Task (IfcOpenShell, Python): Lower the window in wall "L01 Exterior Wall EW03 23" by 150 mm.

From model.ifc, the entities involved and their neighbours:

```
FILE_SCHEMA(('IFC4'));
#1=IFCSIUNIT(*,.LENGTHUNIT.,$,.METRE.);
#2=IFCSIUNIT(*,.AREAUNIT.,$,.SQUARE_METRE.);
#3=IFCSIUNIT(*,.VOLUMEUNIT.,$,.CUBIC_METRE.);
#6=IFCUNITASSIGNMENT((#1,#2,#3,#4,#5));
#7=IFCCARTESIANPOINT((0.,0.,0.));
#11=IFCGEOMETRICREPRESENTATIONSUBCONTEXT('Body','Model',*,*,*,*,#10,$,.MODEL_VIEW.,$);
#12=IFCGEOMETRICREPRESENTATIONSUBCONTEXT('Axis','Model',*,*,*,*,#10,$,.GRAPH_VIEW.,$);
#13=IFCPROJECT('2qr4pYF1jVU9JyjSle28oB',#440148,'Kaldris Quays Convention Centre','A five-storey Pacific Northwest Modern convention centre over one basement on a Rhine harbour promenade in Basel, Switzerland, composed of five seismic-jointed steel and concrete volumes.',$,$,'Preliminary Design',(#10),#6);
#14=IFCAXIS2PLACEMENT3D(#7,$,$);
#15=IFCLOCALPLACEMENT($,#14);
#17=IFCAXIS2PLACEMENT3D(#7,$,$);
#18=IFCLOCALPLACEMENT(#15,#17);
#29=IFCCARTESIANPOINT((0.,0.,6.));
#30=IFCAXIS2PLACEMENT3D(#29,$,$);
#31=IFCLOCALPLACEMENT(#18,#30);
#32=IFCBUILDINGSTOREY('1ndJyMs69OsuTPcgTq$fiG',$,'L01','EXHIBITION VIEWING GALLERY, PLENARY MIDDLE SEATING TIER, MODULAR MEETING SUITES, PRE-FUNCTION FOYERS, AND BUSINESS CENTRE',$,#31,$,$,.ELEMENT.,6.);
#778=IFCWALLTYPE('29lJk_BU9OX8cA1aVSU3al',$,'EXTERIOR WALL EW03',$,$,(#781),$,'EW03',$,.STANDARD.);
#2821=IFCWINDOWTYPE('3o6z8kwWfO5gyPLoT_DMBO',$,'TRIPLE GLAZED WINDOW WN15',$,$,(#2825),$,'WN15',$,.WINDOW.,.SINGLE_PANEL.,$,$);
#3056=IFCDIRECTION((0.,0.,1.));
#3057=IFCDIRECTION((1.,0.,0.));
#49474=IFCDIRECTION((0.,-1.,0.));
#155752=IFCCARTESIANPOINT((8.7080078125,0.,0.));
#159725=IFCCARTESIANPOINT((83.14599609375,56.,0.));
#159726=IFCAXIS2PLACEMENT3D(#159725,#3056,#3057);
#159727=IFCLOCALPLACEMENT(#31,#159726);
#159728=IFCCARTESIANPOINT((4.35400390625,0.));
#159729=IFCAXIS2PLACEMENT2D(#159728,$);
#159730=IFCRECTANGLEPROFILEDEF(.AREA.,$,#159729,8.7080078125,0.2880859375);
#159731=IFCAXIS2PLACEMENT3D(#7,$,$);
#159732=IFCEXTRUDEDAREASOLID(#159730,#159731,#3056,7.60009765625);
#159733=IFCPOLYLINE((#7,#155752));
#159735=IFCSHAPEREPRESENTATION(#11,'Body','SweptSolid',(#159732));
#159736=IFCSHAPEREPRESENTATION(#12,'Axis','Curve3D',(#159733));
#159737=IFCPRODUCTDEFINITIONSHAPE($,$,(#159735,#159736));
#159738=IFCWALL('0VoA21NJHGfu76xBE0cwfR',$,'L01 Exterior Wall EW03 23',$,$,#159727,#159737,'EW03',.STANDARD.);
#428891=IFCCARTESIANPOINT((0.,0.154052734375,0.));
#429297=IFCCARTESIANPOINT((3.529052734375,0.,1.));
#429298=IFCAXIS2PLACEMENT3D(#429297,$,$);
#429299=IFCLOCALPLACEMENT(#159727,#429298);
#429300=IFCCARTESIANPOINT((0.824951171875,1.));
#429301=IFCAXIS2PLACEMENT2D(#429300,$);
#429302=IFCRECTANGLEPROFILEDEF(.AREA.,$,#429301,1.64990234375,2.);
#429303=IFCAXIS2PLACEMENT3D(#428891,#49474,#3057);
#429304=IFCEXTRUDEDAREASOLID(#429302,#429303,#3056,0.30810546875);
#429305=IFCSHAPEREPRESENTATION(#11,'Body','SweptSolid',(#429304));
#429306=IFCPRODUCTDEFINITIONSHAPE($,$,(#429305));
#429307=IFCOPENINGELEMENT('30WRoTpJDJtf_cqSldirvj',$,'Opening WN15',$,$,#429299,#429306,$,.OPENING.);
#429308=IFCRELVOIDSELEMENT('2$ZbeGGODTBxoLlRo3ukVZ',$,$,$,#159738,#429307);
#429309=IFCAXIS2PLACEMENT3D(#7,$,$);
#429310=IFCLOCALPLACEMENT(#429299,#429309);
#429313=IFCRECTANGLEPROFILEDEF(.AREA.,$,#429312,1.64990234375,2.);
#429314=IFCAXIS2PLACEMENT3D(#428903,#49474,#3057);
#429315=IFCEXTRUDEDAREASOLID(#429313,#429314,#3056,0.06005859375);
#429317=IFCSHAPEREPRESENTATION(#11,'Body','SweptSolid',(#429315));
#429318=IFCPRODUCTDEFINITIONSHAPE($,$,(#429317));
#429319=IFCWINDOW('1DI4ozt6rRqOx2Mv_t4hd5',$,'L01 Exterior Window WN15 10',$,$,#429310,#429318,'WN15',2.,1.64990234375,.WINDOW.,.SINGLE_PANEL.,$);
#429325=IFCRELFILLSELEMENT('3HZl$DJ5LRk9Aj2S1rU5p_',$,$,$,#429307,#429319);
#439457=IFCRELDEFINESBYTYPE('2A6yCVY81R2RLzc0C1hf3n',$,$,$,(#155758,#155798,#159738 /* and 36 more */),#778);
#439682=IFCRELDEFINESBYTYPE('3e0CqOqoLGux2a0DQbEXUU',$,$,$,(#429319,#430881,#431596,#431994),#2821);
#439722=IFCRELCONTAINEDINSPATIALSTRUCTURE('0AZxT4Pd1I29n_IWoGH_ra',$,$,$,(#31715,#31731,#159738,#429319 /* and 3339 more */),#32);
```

```python
import numpy as np
import ifcopenshell
import ifcopenshell.api.geometry
import ifcopenshell.util.placement
import ifcopenshell.util.unit

model = ifcopenshell.open("model.ifc")
unit_scale = ifcopenshell.util.unit.calculate_unit_scale(model)

window = model.by_id(429319)
opening = window.FillsVoids[0].RelatingOpeningElement
dz = -0.15 / unit_scale

shift = np.array([0.0, 0.0, dz])
# The window is placed relative to its opening, so it follows when the opening moves.
matrix = ifcopenshell.util.placement.get_local_placement(opening.ObjectPlacement)
matrix[:3, 3] += shift
ifcopenshell.api.geometry.edit_object_placement(
    model, product=opening, matrix=matrix, is_si=False, should_transform_children=True
)

print(f"moved by {dz * unit_scale:+.3f} m")

model.write("model_updated.ifc")
```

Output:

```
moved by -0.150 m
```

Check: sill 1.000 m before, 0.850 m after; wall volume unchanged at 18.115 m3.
